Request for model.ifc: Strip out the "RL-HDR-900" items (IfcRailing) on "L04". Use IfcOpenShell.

First a look at what the model holds.

```python
import ifcopenshell
import ifcopenshell.util.element

model = ifcopenshell.open("model.ifc")
print(model.schema)
storey = next(s for s in model.by_type("IfcBuildingStorey") if s.Name == "L04")
railings = [e for e in ifcopenshell.util.element.get_decomposition(storey) if e.is_a("IfcRailing")]
seen = {}
for e in railings:
    element_type = ifcopenshell.util.element.get_type(e)
    name = element_type.Name if element_type not in (None, e) else None
    seen[name] = seen.get(name, 0) + 1
for name, count in sorted(seen.items(), key=str):
    print(count, "x", name)
```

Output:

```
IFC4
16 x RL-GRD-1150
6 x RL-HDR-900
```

```python
import ifcopenshell
import ifcopenshell.api.root
import ifcopenshell.util.element

model = ifcopenshell.open("model.ifc")

storey = next(s for s in model.by_type("IfcBuildingStorey") if s.Name == "L04")
railings = [e for e in ifcopenshell.util.element.get_decomposition(storey) if e.is_a("IfcRailing")]
targets = [e for e in railings if (t := ifcopenshell.util.element.get_type(e)) not in (None, e) and t.Name == "RL-HDR-900"]

for e in targets:
    ifcopenshell.api.root.remove_product(model, product=e)
print(len(targets), "removed")

model.write("model_edited.ifc")
```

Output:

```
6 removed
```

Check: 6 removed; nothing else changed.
